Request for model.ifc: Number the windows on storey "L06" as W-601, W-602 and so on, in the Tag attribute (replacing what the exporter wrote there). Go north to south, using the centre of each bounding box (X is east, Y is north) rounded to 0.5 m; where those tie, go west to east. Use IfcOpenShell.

First a look at what the model holds.

```python
import ifcopenshell
import ifcopenshell.util.element
import ifcopenshell.util.placement

model = ifcopenshell.open("model.ifc")
print(model.schema)
storey = next(s for s in model.by_type("IfcBuildingStorey") if s.Name == "L06")
windows = [e for e in ifcopenshell.util.element.get_decomposition(storey) if e.is_a("IfcWindow")]
for e in sorted(windows, key=lambda e: e.id()):
    origin = ifcopenshell.util.placement.get_local_placement(e.ObjectPlacement)[:3, 3]
    print(e.id(), e.Tag, e.Name, origin.round(2) + 0.0, sep=" | ")
```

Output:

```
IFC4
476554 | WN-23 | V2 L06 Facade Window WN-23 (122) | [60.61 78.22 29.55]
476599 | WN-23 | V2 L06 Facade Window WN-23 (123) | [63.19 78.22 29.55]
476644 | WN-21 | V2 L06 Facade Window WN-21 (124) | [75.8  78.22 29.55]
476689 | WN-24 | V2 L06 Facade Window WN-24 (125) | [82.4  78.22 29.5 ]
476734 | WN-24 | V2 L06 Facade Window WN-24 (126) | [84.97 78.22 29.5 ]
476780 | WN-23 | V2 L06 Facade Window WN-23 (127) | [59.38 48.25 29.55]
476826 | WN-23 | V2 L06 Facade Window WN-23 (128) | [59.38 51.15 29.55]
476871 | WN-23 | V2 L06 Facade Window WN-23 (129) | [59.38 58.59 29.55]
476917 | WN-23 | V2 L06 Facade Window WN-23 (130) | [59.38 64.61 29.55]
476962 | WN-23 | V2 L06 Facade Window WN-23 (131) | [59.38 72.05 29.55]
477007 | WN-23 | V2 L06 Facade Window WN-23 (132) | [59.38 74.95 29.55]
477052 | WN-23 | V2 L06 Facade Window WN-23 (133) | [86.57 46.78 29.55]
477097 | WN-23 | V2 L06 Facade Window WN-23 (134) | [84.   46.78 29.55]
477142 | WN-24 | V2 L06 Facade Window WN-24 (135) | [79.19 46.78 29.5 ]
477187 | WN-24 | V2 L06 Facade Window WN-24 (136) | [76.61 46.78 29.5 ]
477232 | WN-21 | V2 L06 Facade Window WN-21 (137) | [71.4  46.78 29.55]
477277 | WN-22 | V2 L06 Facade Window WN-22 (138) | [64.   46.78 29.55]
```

```python
import ifcopenshell
import ifcopenshell.geom
import ifcopenshell.util.element
import ifcopenshell.util.shape

model = ifcopenshell.open("model.ifc")
settings = ifcopenshell.geom.settings()
settings.set("use-world-coords", True)


def centre(element):
    shape = ifcopenshell.geom.create_shape(settings, element)
    return ifcopenshell.util.shape.get_bbox_centroid(shape.geometry)


storey = next(s for s in model.by_type("IfcBuildingStorey") if s.Name == "L06")
windows = [e for e in ifcopenshell.util.element.get_decomposition(storey) if e.is_a("IfcWindow")]

# Insertion points can sit at a corner or the storey origin, so sort by the geometry (in metres).
centres = {e: centre(e) for e in windows}
windows.sort(key=lambda e: (-round(centres[e][1] / 0.5), centres[e][0]))

for i, e in enumerate(windows, start=1):
    number = f"W-6{i:02d}"
    e.Tag = number
    print(e.id(), number)

model.write("model_rev.ifc")
```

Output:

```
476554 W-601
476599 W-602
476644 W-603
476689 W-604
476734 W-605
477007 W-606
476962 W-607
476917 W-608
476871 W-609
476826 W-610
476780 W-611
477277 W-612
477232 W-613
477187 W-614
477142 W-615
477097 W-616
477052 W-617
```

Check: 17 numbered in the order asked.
